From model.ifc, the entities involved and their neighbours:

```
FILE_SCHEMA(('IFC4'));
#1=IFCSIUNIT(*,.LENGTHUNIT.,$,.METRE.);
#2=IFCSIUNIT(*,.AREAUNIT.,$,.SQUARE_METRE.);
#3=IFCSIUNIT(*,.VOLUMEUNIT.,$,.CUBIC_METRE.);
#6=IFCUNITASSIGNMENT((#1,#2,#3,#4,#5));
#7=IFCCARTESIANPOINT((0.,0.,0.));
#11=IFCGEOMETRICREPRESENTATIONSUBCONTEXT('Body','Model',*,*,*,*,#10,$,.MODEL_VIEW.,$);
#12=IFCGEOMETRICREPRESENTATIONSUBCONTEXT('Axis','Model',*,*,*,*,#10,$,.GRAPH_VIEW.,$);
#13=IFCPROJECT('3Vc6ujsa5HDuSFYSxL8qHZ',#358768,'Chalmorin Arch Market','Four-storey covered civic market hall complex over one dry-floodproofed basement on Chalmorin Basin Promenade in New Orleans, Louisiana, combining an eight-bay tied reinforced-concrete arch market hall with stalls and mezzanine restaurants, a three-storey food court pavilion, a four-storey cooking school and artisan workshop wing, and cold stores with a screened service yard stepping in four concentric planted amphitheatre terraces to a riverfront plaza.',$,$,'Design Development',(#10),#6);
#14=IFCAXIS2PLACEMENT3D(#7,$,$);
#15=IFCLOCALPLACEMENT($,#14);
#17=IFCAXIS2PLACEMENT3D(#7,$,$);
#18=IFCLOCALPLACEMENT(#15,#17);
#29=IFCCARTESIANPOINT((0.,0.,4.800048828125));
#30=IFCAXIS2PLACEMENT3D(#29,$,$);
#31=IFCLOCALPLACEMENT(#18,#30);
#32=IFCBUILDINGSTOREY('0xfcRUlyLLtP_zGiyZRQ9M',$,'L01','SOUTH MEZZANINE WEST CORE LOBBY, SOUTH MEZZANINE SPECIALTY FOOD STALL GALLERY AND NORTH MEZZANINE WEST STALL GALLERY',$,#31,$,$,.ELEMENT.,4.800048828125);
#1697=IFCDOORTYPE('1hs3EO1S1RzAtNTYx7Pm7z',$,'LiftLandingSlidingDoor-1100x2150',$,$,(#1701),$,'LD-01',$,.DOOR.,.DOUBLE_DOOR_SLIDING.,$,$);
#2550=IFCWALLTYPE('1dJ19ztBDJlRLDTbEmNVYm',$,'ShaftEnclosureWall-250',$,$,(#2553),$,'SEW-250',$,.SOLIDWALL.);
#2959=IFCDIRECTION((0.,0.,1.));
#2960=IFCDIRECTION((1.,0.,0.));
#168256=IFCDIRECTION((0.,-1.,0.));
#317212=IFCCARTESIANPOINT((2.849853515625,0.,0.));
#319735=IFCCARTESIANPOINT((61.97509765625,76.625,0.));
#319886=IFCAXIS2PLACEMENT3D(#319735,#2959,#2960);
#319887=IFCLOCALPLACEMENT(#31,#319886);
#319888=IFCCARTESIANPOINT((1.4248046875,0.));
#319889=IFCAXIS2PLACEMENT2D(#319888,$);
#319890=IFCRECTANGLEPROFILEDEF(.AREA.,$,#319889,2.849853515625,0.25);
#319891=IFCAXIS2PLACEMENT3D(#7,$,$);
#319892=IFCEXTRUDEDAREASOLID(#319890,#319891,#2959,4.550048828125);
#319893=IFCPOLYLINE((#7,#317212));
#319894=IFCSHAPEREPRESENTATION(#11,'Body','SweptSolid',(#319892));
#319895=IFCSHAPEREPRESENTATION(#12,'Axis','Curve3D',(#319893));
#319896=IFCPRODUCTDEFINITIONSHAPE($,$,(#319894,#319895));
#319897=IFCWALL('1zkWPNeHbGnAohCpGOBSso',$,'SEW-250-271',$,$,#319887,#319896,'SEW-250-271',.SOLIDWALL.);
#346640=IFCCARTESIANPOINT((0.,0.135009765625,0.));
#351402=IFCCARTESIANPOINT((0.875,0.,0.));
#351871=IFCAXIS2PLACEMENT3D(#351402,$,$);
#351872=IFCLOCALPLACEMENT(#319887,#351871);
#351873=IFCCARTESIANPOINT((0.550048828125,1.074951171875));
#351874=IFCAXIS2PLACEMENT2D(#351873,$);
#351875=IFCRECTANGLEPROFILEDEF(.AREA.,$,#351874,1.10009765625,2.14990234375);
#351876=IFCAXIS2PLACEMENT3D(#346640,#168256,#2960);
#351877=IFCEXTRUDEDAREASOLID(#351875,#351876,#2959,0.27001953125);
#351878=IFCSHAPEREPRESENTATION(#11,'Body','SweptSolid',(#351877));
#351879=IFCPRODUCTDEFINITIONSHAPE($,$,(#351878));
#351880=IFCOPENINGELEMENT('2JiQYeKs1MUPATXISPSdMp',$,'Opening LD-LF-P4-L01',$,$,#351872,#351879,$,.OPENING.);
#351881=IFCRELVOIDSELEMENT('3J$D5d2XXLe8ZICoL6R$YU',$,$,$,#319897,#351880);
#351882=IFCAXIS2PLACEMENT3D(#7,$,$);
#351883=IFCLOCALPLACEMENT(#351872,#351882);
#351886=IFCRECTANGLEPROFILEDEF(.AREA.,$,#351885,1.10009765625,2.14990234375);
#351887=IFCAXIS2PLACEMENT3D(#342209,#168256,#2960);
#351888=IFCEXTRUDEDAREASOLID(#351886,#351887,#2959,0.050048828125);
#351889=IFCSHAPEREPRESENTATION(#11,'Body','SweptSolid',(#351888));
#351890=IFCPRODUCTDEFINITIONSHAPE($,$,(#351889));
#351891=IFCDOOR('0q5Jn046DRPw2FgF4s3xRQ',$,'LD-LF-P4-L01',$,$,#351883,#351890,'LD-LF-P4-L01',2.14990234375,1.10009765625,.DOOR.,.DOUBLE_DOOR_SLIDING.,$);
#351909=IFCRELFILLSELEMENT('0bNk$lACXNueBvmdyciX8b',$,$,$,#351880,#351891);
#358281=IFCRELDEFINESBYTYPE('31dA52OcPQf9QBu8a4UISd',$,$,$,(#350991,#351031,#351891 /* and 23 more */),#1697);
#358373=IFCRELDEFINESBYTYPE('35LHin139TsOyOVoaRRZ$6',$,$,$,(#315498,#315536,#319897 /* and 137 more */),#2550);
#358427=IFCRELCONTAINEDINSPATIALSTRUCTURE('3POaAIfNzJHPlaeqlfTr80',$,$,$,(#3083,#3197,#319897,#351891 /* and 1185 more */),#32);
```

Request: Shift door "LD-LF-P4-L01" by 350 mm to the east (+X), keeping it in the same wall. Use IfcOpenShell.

```python
import ifcopenshell
import ifcopenshell.api.geometry
import ifcopenshell.util.placement
import ifcopenshell.util.unit

model = ifcopenshell.open("model.ifc")
unit_scale = ifcopenshell.util.unit.calculate_unit_scale(model)

door = model.by_id(351891)
opening = door.FillsVoids[0].RelatingOpeningElement
wall = opening.VoidsElements[0].RelatingBuildingElement

wall_matrix = ifcopenshell.util.placement.get_local_placement(wall.ObjectPlacement)
shift = wall_matrix[:3, 0] * 0.35 / unit_scale
before = ifcopenshell.util.placement.get_local_placement(door.ObjectPlacement)[:3, 3].copy()

# The door is placed relative to its opening, so it follows when the opening moves.
matrix = ifcopenshell.util.placement.get_local_placement(opening.ObjectPlacement)
matrix[:3, 3] += shift
ifcopenshell.api.geometry.edit_object_placement(
    model, product=opening, matrix=matrix, is_si=False, should_transform_children=True
)

after = ifcopenshell.util.placement.get_local_placement(door.ObjectPlacement)[:3, 3]
print("door moved by", (after - before).round(3) + 0.0)

model.write("model-out.ifc")
```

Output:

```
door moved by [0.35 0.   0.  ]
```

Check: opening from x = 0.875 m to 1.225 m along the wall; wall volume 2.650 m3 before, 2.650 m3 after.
